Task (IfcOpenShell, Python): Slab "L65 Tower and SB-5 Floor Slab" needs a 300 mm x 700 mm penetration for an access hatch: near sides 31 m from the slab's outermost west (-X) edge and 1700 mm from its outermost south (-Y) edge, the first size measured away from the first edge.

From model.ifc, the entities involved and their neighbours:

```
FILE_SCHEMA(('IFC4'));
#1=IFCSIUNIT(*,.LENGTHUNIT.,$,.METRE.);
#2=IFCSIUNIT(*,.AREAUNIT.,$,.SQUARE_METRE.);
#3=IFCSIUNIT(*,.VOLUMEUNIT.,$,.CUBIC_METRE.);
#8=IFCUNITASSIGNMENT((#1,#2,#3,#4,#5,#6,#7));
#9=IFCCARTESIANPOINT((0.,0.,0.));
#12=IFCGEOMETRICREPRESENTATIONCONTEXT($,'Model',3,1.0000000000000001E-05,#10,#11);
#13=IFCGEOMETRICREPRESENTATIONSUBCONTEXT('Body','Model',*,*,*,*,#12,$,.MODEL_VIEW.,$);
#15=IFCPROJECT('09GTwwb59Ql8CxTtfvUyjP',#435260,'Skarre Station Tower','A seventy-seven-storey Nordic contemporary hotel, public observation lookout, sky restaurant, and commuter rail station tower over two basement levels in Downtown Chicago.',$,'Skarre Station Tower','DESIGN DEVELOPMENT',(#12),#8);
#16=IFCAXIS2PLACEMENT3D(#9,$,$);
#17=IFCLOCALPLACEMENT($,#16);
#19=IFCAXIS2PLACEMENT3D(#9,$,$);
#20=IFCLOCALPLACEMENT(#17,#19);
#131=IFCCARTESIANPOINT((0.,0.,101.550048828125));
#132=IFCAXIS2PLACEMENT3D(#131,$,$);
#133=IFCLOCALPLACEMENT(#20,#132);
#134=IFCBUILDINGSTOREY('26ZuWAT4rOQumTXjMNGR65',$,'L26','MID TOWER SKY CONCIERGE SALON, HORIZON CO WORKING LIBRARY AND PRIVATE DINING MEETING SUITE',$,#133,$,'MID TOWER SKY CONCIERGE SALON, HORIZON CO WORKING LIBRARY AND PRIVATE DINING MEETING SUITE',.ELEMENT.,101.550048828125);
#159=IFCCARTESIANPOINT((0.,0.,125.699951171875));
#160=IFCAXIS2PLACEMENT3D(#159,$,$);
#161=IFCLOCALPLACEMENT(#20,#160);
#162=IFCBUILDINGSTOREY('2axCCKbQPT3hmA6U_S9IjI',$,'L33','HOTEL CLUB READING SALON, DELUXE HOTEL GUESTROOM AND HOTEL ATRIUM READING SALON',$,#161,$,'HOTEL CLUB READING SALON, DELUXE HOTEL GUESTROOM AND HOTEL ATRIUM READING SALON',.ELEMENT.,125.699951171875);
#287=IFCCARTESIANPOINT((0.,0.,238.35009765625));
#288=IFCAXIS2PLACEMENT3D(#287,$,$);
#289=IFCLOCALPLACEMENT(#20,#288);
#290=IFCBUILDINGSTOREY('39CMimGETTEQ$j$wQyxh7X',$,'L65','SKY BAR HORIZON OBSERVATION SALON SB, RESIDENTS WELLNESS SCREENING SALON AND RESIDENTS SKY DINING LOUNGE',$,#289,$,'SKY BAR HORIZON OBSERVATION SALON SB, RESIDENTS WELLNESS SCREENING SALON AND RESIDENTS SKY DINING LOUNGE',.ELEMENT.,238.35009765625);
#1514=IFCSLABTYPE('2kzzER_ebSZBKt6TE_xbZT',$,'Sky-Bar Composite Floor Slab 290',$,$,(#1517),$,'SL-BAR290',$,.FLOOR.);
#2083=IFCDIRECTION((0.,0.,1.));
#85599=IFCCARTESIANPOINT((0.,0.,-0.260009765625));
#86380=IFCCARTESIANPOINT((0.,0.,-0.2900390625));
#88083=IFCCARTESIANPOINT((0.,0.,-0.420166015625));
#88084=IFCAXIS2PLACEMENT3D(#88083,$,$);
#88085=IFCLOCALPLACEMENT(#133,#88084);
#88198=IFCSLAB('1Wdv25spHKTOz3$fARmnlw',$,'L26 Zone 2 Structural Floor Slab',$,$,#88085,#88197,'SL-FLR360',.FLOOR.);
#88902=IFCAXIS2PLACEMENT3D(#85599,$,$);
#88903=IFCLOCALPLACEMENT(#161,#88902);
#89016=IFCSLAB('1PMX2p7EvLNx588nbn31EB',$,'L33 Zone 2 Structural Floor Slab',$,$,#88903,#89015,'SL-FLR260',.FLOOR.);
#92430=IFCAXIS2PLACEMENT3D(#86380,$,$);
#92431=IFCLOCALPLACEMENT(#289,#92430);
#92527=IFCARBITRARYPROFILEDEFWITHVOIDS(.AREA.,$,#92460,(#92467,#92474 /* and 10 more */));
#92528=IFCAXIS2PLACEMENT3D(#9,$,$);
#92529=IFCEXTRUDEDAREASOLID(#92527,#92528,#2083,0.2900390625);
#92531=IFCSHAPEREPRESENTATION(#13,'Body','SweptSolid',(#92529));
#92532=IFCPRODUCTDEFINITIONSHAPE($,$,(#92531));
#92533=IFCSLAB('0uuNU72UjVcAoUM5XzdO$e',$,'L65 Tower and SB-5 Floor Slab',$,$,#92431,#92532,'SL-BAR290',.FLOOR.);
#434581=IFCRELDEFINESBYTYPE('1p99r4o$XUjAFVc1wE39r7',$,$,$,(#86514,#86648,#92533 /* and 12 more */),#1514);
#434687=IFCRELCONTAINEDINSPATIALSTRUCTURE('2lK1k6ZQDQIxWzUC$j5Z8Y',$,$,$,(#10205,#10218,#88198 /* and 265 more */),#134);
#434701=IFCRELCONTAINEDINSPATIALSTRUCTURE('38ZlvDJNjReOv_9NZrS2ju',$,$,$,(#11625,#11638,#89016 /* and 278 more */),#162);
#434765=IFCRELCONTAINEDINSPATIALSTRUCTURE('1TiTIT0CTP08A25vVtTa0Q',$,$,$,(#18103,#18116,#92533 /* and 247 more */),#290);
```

```python
import numpy as np
import ifcopenshell
import ifcopenshell.api.feature
import ifcopenshell.api.geometry
import ifcopenshell.api.root
import ifcopenshell.geom
import ifcopenshell.util.placement
import ifcopenshell.util.representation
import ifcopenshell.util.shape
import ifcopenshell.util.unit

model = ifcopenshell.open("model.ifc")
unit_scale = ifcopenshell.util.unit.calculate_unit_scale(model)
settings = ifcopenshell.geom.settings()


def volume(element):
    """Net volume in cubic metres, openings subtracted."""
    shape = ifcopenshell.geom.create_shape(settings, element)
    return ifcopenshell.util.shape.get_volume(shape.geometry)


slab = model.by_guid("0uuNU72UjVcAoUM5XzdO$e")
before = volume(slab)

# Extent in the slab's own axes, in metres. The edges named are its -X and -Y sides.
slab_shape = ifcopenshell.geom.create_shape(settings, slab)
vertices = ifcopenshell.util.shape.get_vertices(slab_shape.geometry)
x_min, y_min, bottom = vertices.min(axis=0)
top = vertices[:, 2].max()

opening = ifcopenshell.api.root.create_entity(model, ifc_class="IfcOpeningElement", name="Access hatch opening", predefined_type="OPENING")
context = ifcopenshell.util.representation.get_context(model, "Model", "Body", "MODEL_VIEW")
width, depth = 0.3, 0.7
outline = [(0.0, 0.0), (width, 0.0), (width, depth), (0.0, depth), (0.0, 0.0)]
# Overshoot both faces by 50 mm so the cut is clean.
shape = ifcopenshell.api.geometry.add_slab_representation(
    model, context=context, depth=top - bottom + 0.1, polyline=outline
)
ifcopenshell.api.geometry.assign_representation(model, product=opening, representation=shape)

matrix = ifcopenshell.util.placement.get_local_placement(slab.ObjectPlacement)
matrix[:, 3] = matrix @ np.append(np.array([x_min + 31, y_min + 1.7, bottom - 0.05]) / unit_scale, 1.0)
ifcopenshell.api.geometry.edit_object_placement(model, product=opening, matrix=matrix, is_si=False)
ifcopenshell.api.feature.add_feature(model, feature=opening, element=slab)

after = volume(slab)

print(f"slab volume {before:.3f} -> {after:.3f} m3")

model.write("model-out.ifc")
```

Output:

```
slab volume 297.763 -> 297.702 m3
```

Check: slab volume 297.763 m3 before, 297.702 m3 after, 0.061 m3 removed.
